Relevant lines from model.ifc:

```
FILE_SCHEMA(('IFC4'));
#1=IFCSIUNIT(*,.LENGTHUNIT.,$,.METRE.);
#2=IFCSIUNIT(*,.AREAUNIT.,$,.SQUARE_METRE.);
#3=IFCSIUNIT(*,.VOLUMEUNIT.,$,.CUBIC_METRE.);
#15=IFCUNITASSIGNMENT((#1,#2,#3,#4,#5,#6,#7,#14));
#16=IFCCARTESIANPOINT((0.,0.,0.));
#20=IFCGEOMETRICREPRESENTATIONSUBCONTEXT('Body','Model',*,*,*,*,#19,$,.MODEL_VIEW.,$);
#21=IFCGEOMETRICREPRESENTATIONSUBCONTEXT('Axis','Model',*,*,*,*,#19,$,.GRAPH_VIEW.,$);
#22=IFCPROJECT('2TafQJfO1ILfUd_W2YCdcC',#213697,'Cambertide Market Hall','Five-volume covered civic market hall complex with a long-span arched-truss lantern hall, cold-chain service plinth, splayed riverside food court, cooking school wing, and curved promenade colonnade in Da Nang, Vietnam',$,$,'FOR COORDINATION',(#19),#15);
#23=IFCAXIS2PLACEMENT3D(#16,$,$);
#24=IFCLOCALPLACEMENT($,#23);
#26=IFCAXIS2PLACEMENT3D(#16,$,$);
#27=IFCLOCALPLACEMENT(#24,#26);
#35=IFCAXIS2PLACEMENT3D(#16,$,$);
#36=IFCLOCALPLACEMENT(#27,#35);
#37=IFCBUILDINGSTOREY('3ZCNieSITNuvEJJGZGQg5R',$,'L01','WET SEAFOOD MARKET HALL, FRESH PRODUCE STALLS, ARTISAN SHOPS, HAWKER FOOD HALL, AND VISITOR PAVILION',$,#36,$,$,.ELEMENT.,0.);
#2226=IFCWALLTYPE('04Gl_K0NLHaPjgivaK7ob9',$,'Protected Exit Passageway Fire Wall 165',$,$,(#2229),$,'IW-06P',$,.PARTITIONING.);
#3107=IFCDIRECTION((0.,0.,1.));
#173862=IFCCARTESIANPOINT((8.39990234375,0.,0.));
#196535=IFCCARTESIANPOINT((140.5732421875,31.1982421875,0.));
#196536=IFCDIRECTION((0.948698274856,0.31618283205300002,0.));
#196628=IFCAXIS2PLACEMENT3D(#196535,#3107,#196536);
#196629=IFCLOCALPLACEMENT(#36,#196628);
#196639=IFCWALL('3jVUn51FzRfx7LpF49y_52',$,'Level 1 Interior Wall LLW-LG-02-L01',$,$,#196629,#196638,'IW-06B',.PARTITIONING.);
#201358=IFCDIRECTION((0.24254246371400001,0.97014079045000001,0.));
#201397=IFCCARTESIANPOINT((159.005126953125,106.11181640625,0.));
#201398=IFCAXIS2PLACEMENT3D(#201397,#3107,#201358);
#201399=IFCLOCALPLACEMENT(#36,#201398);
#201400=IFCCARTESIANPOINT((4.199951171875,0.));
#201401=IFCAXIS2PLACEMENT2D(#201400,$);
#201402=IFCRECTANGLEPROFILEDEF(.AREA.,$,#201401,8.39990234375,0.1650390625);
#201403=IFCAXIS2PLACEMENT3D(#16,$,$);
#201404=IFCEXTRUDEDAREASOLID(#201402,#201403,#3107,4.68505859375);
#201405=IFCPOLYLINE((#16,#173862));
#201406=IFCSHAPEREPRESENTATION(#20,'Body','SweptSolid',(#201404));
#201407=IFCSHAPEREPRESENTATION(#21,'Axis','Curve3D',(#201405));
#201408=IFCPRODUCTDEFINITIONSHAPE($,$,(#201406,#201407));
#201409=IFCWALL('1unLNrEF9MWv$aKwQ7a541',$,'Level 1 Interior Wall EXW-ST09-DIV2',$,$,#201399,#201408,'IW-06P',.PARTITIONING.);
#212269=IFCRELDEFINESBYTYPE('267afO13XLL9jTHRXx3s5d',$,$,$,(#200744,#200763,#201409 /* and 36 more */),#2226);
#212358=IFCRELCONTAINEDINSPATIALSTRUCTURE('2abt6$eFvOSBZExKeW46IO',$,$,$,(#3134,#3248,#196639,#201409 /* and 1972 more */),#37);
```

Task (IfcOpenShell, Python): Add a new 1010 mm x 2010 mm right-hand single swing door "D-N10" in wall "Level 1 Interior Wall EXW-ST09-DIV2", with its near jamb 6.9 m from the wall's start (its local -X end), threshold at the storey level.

```python
import numpy as np
import ifcopenshell
import ifcopenshell.api.feature
import ifcopenshell.api.geometry
import ifcopenshell.api.root
import ifcopenshell.api.spatial
import ifcopenshell.geom
import ifcopenshell.util.element
import ifcopenshell.util.placement
import ifcopenshell.util.representation
import ifcopenshell.util.shape
import ifcopenshell.util.unit

model = ifcopenshell.open("model.ifc")
unit_scale = ifcopenshell.util.unit.calculate_unit_scale(model)
settings = ifcopenshell.geom.settings()


def volume(element):
    """Net volume in cubic metres, openings subtracted."""
    shape = ifcopenshell.geom.create_shape(settings, element)
    return ifcopenshell.util.shape.get_volume(shape.geometry)


wall = model.by_guid("1unLNrEF9MWv$aKwQ7a541")
storey = ifcopenshell.util.element.get_container(wall, ifc_class="IfcBuildingStorey")
context = ifcopenshell.util.representation.get_context(model, "Model", "Body", "MODEL_VIEW")
before = volume(wall)

width, height, from_end, sill = 1.01, 2.01, 6.9, 0.0  # metres

# The wall runs along its own X axis, and the end named is its -X end.
wall_shape = ifcopenshell.geom.create_shape(settings, wall)
x, y, z = ifcopenshell.util.shape.get_vertices(wall_shape.geometry).T
start = x.min() + from_end
face, thickness = float(y.min()), float(y.max() - y.min())
wall_matrix = ifcopenshell.util.placement.get_local_placement(wall.ObjectPlacement)
level = ifcopenshell.util.placement.get_local_placement(storey.ObjectPlacement)[2, 3]


def in_wall(x, y):
    """Placement at x, y metres in the wall's axes, at sill height."""
    matrix = wall_matrix.copy()
    matrix[:, 3] = wall_matrix @ np.array([x / unit_scale, y / unit_scale, 0.0, 1.0])
    matrix[2, 3] = level + sill / unit_scale
    return matrix


# Opening: a box that overshoots both wall faces by 50 mm.
opening = ifcopenshell.api.root.create_entity(model, ifc_class="IfcOpeningElement", predefined_type="OPENING")
box = ifcopenshell.api.geometry.add_wall_representation(
    model, context=context, length=width, height=height, thickness=thickness + 0.1
)
ifcopenshell.api.geometry.assign_representation(model, product=opening, representation=box)
ifcopenshell.api.geometry.edit_object_placement(model, product=opening, matrix=in_wall(start, face - 0.05), is_si=False)
ifcopenshell.api.feature.add_feature(model, feature=opening, element=wall)

door = ifcopenshell.api.root.create_entity(model, ifc_class="IfcDoor", name="D-N10", predefined_type="DOOR")
door.OverallWidth, door.OverallHeight = width / unit_scale, height / unit_scale
door.OperationType = "SINGLE_SWING_RIGHT"
body = ifcopenshell.api.geometry.add_door_representation(
    model,
    context=context,
    overall_width=door.OverallWidth,
    overall_height=door.OverallHeight,
    operation_type="SINGLE_SWING_RIGHT",
    lining_properties={"LiningDepth": thickness / unit_scale, "ThresholdDepth": thickness / unit_scale},
)
ifcopenshell.api.geometry.assign_representation(model, product=door, representation=body)
ifcopenshell.api.spatial.assign_container(model, products=[door], relating_structure=storey)
ifcopenshell.api.feature.add_filling(model, opening=opening, element=door)

# The lining spans the wall, so the door starts at the wall face.
ifcopenshell.api.geometry.edit_object_placement(model, product=door, matrix=in_wall(start, face), is_si=False)

after = volume(wall)

print(f"wall volume {before:.3f} -> {after:.3f} m3")

model.write("model_updated.ifc")
```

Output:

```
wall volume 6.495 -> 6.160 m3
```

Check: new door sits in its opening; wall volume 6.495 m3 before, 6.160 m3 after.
